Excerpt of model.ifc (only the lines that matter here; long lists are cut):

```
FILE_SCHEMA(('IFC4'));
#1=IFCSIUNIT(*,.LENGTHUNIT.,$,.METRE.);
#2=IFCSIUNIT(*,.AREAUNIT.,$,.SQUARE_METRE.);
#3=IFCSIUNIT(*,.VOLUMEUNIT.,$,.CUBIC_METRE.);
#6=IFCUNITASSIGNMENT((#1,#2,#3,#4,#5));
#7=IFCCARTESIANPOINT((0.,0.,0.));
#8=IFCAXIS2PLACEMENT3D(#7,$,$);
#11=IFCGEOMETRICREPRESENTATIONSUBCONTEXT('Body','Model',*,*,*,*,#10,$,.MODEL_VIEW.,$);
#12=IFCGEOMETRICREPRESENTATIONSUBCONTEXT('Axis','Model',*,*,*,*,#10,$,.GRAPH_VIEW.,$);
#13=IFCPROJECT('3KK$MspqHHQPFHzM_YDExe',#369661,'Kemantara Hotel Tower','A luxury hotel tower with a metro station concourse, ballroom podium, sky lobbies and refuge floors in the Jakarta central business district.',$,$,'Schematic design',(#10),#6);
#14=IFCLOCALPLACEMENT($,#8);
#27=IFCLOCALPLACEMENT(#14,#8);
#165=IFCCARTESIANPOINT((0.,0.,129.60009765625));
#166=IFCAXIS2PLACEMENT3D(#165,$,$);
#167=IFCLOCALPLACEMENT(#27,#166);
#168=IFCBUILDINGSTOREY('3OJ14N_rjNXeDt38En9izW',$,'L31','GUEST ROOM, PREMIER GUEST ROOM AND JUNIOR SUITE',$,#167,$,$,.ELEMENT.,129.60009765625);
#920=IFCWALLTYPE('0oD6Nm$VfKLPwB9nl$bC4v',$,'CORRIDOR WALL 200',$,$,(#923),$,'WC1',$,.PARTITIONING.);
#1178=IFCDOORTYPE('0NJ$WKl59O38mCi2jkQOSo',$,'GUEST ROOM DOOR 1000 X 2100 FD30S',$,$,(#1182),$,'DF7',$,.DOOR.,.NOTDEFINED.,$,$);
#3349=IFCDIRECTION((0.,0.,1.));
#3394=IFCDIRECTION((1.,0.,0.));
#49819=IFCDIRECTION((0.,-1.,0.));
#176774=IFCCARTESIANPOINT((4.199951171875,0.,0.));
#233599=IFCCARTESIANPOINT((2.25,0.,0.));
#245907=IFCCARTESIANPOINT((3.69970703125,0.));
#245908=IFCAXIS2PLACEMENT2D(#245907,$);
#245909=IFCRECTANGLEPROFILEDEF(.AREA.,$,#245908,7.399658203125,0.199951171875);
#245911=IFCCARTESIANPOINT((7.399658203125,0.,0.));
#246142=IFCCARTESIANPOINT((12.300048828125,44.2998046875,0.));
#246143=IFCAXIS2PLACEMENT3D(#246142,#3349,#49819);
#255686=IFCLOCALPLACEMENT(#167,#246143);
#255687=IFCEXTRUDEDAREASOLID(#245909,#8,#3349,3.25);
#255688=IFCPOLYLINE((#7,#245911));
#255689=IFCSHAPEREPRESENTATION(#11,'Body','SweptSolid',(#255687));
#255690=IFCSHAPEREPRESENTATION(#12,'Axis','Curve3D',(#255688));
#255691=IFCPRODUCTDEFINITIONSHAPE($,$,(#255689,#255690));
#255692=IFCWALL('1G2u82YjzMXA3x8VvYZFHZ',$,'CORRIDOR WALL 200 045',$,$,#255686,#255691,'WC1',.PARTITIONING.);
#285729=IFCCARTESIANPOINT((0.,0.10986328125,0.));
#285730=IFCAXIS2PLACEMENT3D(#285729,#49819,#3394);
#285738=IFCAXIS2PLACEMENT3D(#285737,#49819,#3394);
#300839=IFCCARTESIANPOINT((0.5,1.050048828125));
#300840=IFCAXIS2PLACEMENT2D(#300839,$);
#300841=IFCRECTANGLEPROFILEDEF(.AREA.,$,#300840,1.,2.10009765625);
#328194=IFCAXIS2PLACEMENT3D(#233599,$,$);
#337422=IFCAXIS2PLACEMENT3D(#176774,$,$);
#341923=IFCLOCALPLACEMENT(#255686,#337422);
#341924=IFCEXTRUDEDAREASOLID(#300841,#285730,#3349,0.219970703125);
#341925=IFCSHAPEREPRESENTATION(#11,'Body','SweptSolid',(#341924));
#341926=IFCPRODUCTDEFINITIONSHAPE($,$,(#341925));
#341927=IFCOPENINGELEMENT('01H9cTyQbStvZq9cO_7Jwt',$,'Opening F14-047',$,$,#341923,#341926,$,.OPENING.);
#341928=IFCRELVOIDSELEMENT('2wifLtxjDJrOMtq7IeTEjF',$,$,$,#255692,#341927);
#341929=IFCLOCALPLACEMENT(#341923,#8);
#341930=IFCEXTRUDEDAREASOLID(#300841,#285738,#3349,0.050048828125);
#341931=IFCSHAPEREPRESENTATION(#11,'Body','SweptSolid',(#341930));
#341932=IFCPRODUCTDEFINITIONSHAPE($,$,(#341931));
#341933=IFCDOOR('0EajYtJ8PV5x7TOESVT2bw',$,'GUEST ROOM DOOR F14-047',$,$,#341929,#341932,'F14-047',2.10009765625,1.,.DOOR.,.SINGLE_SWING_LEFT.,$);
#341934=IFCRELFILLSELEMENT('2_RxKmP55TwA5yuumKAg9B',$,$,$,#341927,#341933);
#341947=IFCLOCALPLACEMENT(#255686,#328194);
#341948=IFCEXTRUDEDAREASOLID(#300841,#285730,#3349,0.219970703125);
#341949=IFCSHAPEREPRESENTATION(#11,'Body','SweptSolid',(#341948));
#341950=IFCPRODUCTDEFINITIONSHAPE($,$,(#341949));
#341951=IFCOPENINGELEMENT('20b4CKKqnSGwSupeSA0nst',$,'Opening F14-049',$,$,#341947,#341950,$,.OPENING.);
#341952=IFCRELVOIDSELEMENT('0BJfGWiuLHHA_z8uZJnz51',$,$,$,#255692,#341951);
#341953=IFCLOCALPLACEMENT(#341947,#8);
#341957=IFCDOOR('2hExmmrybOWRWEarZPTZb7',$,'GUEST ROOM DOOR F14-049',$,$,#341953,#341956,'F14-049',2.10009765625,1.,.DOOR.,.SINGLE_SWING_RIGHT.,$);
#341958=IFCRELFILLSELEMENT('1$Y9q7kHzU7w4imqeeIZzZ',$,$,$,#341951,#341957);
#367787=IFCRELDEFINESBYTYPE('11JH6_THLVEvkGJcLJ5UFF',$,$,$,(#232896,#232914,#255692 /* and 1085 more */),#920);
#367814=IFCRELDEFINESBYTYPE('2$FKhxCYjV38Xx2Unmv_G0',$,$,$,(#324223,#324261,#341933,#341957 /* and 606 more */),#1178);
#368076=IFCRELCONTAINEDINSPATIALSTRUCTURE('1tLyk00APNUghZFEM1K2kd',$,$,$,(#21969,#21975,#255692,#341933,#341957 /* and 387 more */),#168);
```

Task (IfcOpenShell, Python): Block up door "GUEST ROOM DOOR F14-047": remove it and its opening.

```python
import ifcopenshell
import ifcopenshell.api.feature
import ifcopenshell.api.root
import ifcopenshell.geom
import ifcopenshell.util.shape

model = ifcopenshell.open("model.ifc")
settings = ifcopenshell.geom.settings()


def volume(element):
    """Net volume in cubic metres, openings subtracted."""
    shape = ifcopenshell.geom.create_shape(settings, element)
    return ifcopenshell.util.shape.get_volume(shape.geometry)


door = model.by_guid("0EajYtJ8PV5x7TOESVT2bw")
opening = door.FillsVoids[0].RelatingOpeningElement
wall = opening.VoidsElements[0].RelatingBuildingElement
before = volume(wall)

ifcopenshell.api.root.remove_product(model, product=door)
ifcopenshell.api.feature.remove_feature(model, feature=opening)

after = volume(wall)

print(f"wall volume {before:.3f} -> {after:.3f} m3")

model.write("model_updated.ifc")
```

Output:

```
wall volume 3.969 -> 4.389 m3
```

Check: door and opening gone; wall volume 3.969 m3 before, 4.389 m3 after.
